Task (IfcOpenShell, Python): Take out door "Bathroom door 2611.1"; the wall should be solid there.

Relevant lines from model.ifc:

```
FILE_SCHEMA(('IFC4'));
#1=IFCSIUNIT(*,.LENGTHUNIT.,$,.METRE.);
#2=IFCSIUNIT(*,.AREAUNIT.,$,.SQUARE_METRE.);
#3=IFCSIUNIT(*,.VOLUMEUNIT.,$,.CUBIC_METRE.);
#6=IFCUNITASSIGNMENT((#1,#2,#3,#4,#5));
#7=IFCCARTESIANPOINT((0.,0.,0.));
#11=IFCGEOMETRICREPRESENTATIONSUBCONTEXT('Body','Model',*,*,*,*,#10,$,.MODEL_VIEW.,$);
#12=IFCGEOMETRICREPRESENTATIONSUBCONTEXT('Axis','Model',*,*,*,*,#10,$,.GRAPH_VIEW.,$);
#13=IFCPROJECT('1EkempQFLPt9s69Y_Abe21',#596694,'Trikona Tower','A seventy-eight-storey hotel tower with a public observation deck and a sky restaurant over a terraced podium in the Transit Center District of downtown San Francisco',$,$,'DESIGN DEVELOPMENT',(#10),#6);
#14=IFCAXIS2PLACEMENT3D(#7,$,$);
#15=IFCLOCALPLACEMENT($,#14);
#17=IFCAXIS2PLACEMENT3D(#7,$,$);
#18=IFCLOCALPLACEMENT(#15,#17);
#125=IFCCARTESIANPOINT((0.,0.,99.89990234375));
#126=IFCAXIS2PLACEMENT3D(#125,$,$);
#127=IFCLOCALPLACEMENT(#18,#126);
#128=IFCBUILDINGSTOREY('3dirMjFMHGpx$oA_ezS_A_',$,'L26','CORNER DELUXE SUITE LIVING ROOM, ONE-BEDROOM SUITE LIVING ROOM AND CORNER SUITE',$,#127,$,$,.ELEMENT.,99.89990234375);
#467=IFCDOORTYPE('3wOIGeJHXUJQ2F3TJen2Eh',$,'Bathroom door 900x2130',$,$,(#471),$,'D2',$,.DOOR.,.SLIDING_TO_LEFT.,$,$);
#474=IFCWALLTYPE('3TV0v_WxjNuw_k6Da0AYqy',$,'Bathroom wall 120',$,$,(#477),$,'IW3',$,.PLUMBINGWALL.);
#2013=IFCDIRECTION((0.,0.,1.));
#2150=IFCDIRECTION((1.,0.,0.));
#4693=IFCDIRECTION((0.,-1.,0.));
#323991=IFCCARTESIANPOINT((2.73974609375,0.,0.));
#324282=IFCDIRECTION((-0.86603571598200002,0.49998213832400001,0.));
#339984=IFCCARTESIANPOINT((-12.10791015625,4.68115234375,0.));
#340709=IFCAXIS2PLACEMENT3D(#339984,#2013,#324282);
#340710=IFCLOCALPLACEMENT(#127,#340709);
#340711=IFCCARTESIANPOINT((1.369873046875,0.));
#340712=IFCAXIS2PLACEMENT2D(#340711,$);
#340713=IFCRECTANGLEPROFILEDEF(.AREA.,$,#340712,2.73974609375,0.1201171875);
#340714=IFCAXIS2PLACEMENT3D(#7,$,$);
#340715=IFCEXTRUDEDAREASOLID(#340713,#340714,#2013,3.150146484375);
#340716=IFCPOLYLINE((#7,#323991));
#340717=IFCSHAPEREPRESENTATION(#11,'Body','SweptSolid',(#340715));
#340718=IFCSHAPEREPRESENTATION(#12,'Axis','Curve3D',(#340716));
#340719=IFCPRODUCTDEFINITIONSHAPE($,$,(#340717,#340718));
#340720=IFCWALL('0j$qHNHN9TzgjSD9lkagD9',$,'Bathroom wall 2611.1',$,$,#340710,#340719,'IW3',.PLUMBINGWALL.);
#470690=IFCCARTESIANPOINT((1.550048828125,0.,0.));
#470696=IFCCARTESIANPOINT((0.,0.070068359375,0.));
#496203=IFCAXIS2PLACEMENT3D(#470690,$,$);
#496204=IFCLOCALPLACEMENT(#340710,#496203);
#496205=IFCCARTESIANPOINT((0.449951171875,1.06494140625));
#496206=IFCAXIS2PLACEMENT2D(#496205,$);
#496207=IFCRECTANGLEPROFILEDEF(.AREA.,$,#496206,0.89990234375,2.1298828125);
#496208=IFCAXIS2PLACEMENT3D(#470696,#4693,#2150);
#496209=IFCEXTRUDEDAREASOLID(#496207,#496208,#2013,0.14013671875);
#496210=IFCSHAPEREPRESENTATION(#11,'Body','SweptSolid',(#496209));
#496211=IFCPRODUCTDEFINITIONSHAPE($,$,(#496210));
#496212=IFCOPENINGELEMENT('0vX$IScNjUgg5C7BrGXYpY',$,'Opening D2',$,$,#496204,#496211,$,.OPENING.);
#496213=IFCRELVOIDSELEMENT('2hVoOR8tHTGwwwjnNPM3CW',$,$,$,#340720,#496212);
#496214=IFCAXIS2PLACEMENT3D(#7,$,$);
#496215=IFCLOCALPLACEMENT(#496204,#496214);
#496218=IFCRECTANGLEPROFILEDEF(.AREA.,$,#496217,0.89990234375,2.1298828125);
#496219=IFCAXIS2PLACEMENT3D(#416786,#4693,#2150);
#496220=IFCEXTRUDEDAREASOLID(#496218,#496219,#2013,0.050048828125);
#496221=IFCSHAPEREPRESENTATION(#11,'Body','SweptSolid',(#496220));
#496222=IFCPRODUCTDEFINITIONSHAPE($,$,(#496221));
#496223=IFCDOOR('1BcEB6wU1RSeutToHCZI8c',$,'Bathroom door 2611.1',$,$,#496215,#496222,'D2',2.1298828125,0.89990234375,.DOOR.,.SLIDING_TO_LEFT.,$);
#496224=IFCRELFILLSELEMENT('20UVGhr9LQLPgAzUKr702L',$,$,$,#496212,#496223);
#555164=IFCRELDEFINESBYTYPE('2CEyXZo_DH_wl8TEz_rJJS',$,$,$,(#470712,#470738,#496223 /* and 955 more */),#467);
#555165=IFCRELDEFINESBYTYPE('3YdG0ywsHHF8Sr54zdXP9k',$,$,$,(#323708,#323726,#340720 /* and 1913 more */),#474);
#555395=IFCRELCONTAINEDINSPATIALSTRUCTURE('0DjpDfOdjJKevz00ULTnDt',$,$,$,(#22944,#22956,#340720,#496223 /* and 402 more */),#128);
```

```python
import ifcopenshell
import ifcopenshell.api.feature
import ifcopenshell.api.root
import ifcopenshell.geom
import ifcopenshell.util.shape

model = ifcopenshell.open("model.ifc")
settings = ifcopenshell.geom.settings()


def volume(element):
    """Net volume in cubic metres, openings subtracted."""
    shape = ifcopenshell.geom.create_shape(settings, element)
    return ifcopenshell.util.shape.get_volume(shape.geometry)


door = model.by_guid("1BcEB6wU1RSeutToHCZI8c")
opening = door.FillsVoids[0].RelatingOpeningElement
wall = opening.VoidsElements[0].RelatingBuildingElement
before = volume(wall)

ifcopenshell.api.root.remove_product(model, product=door)
ifcopenshell.api.feature.remove_feature(model, feature=opening)

after = volume(wall)

print(f"wall volume {before:.3f} -> {after:.3f} m3")

model.write("model_v2.ifc")
```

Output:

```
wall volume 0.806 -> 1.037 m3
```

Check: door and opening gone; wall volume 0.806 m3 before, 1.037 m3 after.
